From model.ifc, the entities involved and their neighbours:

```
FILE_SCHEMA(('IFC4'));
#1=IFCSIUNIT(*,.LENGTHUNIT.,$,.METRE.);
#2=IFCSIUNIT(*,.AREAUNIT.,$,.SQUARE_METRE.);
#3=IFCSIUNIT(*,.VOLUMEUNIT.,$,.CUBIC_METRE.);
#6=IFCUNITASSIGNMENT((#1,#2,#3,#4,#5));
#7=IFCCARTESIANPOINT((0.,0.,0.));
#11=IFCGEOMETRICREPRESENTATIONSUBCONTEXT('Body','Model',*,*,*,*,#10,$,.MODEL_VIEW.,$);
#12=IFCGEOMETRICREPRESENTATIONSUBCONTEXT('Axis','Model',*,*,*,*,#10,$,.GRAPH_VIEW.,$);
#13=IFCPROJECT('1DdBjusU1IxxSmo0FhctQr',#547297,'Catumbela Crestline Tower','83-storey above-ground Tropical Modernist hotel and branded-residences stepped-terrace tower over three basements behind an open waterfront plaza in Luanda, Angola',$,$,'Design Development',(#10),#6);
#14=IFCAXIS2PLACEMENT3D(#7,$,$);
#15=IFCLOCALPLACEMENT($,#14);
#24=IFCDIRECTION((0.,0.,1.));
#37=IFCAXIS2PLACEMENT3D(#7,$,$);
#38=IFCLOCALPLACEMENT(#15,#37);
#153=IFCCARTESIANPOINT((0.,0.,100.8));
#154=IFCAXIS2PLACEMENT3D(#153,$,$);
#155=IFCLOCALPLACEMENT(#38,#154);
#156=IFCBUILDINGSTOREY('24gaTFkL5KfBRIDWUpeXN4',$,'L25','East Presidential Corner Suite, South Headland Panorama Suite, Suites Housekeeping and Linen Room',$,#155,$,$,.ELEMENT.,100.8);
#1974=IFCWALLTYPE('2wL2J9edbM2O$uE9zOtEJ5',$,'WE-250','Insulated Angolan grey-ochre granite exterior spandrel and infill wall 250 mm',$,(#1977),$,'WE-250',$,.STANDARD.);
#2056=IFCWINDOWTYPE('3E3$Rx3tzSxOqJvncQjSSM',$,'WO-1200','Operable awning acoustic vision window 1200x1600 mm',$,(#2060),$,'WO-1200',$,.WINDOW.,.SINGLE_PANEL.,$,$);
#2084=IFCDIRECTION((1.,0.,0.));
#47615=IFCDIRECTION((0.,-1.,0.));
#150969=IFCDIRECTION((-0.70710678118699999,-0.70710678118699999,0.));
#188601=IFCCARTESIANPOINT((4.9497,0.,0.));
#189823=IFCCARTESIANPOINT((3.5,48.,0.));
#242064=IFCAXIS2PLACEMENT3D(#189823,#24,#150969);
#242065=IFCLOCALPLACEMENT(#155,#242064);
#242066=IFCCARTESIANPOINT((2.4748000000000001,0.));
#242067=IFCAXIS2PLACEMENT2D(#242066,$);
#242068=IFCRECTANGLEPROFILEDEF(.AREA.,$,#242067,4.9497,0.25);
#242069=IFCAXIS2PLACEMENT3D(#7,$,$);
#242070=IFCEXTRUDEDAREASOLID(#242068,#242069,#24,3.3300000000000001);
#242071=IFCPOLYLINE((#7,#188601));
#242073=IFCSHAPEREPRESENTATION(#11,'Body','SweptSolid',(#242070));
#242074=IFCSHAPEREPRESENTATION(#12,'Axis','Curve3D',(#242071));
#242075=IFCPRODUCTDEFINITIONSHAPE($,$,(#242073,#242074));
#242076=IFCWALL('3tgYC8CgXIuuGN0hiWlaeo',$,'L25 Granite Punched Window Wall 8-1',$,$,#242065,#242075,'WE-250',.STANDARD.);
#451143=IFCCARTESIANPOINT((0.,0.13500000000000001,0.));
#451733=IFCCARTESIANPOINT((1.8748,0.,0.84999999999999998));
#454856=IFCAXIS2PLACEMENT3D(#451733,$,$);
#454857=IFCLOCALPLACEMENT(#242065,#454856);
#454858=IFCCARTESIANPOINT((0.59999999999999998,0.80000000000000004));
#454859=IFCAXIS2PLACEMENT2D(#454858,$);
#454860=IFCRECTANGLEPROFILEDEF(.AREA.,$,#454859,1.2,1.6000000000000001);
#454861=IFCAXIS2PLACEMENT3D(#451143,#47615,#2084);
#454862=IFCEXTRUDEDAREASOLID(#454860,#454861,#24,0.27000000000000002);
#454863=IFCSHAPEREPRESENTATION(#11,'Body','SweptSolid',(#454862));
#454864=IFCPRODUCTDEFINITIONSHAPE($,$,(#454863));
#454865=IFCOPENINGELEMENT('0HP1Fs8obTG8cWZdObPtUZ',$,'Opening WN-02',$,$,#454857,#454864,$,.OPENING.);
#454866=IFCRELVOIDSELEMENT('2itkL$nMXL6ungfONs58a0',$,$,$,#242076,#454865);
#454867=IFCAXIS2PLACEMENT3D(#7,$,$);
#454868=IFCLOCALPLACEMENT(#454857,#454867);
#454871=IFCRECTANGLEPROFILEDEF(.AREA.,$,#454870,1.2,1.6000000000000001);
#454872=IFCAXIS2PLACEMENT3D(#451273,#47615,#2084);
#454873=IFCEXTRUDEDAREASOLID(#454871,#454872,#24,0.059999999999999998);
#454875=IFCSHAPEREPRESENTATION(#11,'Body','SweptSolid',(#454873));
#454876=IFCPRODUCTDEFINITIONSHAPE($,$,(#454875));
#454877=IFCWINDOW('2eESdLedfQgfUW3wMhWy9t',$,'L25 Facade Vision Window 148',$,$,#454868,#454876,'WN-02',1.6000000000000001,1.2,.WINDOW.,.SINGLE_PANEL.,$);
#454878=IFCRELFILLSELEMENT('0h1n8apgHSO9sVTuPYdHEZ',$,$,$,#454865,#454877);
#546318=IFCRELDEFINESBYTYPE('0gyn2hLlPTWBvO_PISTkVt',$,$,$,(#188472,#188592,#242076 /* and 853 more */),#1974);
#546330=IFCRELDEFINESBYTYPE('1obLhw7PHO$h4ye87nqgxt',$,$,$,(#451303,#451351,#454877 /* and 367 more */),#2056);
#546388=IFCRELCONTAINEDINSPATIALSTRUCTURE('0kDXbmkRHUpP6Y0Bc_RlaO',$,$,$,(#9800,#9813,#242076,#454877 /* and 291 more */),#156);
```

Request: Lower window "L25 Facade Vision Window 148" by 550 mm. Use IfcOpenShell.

```python
import numpy as np
import ifcopenshell
import ifcopenshell.api.geometry
import ifcopenshell.util.placement
import ifcopenshell.util.unit

model = ifcopenshell.open("model.ifc")
unit_scale = ifcopenshell.util.unit.calculate_unit_scale(model)

window = model.by_id(454877)
opening = window.FillsVoids[0].RelatingOpeningElement
dz = -0.55

shift = np.array([0.0, 0.0, dz])
# The window is placed relative to its opening, so it follows when the opening moves.
matrix = ifcopenshell.util.placement.get_local_placement(opening.ObjectPlacement)
matrix[:3, 3] += shift
ifcopenshell.api.geometry.edit_object_placement(
    model, product=opening, matrix=matrix, is_si=False, should_transform_children=True
)

print(f"moved by {dz * unit_scale:+.3f} m")

model.write("model_edited.ifc")
```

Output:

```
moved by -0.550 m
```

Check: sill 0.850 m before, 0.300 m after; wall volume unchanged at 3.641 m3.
